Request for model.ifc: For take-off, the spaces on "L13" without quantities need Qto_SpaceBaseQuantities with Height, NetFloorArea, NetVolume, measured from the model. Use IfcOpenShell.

First a look at what the model holds.

```python
import ifcopenshell
import ifcopenshell.util.element
import ifcopenshell.util.unit

model = ifcopenshell.open("model.ifc")
print(model.schema)
for unit_type in ("LENGTHUNIT", "AREAUNIT", "VOLUMEUNIT"):
    print(unit_type, ifcopenshell.util.unit.calculate_unit_scale(model, unit_type))
storey = next(s for s in model.by_type("IfcBuildingStorey") if s.Name == "L13")
spaces = [e for e in ifcopenshell.util.element.get_decomposition(storey) if e.is_a("IfcSpace")]
for e in sorted(spaces, key=lambda e: e.id()):
    print(e.id(), e.is_a(), e.Name, list(ifcopenshell.util.element.get_psets(e, qtos_only=True)), sep=" | ")
```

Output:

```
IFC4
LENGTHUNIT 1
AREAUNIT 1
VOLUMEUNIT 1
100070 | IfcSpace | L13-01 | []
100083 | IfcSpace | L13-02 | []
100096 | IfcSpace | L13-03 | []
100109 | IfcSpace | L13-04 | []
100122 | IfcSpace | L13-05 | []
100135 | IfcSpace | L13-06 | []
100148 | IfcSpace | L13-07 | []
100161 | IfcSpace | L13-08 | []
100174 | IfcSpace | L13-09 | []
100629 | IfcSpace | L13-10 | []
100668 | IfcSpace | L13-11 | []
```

```python
import ifcopenshell
import ifcopenshell.api.pset
import ifcopenshell.geom
import ifcopenshell.util.element
import ifcopenshell.util.shape
import ifcopenshell.util.unit

model = ifcopenshell.open("model.ifc")
unit_scale = ifcopenshell.util.unit.calculate_unit_scale(model)
area_scale = ifcopenshell.util.unit.calculate_unit_scale(model, "AREAUNIT")
volume_scale = ifcopenshell.util.unit.calculate_unit_scale(model, "VOLUMEUNIT")
settings = ifcopenshell.geom.settings()

storey = next(s for s in model.by_type("IfcBuildingStorey") if s.Name == "L13")
spaces = [e for e in ifcopenshell.util.element.get_decomposition(storey) if e.is_a("IfcSpace")]

for e in sorted(spaces, key=lambda e: e.id()):
    if ifcopenshell.util.element.get_psets(e, qtos_only=True, should_inherit=False):
        continue
    # Geometry comes back in metres, in the element's own axes.
    shape = ifcopenshell.geom.create_shape(settings, e)
    values = {
        "Height": ifcopenshell.util.shape.get_z(shape.geometry) / unit_scale,
        "NetFloorArea": ifcopenshell.util.shape.get_footprint_area(shape.geometry) / area_scale,
        "NetVolume": ifcopenshell.util.shape.get_volume(shape.geometry) / volume_scale,
    }
    qto = ifcopenshell.api.pset.add_qto(model, product=e, name="Qto_SpaceBaseQuantities")
    ifcopenshell.api.pset.edit_qto(model, qto=qto, properties=values)
    print(e.id(), {k: round(v, 3) for k, v in values.items()})

model.write("model_rev.ifc")
```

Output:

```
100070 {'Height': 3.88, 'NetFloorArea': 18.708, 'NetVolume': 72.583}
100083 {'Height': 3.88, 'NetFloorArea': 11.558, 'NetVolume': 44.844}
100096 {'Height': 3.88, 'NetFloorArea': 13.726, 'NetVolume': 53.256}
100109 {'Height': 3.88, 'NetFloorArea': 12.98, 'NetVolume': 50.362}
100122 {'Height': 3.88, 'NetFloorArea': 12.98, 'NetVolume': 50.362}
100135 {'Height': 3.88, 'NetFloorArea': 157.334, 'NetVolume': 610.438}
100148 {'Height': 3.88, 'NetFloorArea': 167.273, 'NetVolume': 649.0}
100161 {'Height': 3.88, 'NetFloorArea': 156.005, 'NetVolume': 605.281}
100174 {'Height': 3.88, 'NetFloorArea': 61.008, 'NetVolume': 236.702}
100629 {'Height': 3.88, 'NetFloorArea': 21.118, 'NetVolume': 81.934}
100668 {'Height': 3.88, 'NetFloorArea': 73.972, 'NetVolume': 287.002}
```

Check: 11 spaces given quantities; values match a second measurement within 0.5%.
